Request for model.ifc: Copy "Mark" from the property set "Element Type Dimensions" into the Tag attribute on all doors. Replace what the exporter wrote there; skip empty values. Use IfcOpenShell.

First a look at what the model holds.

```python
import ifcopenshell
import ifcopenshell.util.element

model = ifcopenshell.open("model.ifc")
print(model.schema)
doors = model.by_type("IfcDoor")
print(len(doors), "doors")
for e in doors[:8]:
    source = ifcopenshell.util.element.get_pset(e, "Element Type Dimensions", "Mark")
    target = e.Tag
    print(e.id(), repr(source), repr(target), sep=" | ")
```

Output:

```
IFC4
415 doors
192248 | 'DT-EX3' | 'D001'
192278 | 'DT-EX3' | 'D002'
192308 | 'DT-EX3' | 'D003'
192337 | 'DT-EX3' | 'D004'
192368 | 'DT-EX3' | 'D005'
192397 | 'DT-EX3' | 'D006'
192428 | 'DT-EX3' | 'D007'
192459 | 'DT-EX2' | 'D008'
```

```python
import ifcopenshell
import ifcopenshell.util.element

model = ifcopenshell.open("model.ifc")

count = 0
for e in model.by_type("IfcDoor"):
    value = ifcopenshell.util.element.get_pset(e, "Element Type Dimensions", "Mark")
    current = e.Tag
    if not value or not value.strip() or current == value:
        continue
    e.Tag = value
    count += 1

print(count, "doors updated")

model.write("model-out.ifc")
```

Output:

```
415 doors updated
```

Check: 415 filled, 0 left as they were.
